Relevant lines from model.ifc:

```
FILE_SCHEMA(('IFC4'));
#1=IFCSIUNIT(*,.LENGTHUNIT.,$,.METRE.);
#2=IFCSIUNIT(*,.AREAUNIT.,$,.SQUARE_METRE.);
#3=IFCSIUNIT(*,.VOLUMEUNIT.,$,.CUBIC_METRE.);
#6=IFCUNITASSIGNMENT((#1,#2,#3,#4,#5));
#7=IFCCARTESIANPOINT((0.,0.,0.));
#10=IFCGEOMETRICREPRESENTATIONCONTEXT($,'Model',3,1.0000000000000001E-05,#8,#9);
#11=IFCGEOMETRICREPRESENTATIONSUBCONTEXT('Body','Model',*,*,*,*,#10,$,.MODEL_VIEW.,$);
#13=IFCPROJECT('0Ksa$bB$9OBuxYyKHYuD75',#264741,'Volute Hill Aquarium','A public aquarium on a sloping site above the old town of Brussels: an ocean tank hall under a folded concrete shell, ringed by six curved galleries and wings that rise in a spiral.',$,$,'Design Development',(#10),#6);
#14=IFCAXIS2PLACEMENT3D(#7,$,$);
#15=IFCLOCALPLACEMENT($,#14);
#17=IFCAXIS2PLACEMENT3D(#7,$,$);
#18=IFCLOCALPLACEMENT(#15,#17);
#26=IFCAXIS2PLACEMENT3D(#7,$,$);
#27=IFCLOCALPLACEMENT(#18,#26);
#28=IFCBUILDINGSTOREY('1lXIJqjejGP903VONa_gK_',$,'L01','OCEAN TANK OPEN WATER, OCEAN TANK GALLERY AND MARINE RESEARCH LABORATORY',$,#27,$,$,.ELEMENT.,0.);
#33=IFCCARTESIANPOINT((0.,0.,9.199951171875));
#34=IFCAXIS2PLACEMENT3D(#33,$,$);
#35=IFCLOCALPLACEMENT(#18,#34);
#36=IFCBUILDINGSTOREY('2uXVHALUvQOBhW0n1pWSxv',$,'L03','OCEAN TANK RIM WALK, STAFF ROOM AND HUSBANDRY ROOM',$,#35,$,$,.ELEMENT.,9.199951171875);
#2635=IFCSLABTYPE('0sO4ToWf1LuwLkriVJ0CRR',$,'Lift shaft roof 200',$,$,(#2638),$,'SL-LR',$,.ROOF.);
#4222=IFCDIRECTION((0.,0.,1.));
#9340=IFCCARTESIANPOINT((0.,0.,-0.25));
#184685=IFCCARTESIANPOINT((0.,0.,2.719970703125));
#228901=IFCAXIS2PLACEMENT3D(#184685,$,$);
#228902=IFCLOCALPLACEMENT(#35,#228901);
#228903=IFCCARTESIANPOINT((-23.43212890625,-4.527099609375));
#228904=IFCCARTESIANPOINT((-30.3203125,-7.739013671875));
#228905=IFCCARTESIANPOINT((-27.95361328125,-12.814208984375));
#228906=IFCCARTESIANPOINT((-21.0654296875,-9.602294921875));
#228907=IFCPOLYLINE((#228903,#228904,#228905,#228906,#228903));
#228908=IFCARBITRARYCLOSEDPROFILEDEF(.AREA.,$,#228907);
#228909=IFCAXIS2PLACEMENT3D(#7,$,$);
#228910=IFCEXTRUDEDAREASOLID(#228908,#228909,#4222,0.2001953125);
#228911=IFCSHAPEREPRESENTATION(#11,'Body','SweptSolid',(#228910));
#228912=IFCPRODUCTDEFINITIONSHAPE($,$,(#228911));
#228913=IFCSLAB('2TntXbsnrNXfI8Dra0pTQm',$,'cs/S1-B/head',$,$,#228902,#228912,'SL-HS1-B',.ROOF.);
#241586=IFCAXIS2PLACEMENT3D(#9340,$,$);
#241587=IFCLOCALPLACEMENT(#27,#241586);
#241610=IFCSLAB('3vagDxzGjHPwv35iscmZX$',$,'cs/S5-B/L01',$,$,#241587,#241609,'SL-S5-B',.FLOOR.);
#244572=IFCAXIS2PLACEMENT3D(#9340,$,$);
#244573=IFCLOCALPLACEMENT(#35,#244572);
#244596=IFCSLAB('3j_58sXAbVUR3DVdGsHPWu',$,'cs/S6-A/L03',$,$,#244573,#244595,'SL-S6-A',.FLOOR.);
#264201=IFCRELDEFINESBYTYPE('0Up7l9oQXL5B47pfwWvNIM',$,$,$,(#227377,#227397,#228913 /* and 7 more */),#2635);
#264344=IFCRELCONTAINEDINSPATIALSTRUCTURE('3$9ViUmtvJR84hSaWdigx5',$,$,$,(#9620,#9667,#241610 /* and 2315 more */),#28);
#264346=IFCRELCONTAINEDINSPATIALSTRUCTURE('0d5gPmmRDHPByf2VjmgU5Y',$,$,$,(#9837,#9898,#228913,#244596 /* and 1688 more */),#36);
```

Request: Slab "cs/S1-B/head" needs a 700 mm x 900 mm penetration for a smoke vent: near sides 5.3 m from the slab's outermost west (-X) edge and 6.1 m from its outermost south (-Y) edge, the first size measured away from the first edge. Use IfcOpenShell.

```python
import numpy as np
import ifcopenshell
import ifcopenshell.api.feature
import ifcopenshell.api.geometry
import ifcopenshell.api.root
import ifcopenshell.geom
import ifcopenshell.util.placement
import ifcopenshell.util.representation
import ifcopenshell.util.shape
import ifcopenshell.util.unit

model = ifcopenshell.open("model.ifc")
unit_scale = ifcopenshell.util.unit.calculate_unit_scale(model)
settings = ifcopenshell.geom.settings()


def volume(element):
    """Net volume in cubic metres, openings subtracted."""
    shape = ifcopenshell.geom.create_shape(settings, element)
    return ifcopenshell.util.shape.get_volume(shape.geometry)


slab = model.by_id(228913)
before = volume(slab)

# Extent in the slab's own axes, in metres. The edges named are its -X and -Y sides.
slab_shape = ifcopenshell.geom.create_shape(settings, slab)
vertices = ifcopenshell.util.shape.get_vertices(slab_shape.geometry)
x_min, y_min, bottom = vertices.min(axis=0)
top = vertices[:, 2].max()

opening = ifcopenshell.api.root.create_entity(model, ifc_class="IfcOpeningElement", name="Smoke vent opening", predefined_type="OPENING")
context = ifcopenshell.util.representation.get_context(model, "Model", "Body", "MODEL_VIEW")
width, depth = 0.7, 0.9
outline = [(0.0, 0.0), (width, 0.0), (width, depth), (0.0, depth), (0.0, 0.0)]
# Overshoot both faces by 50 mm so the cut is clean.
shape = ifcopenshell.api.geometry.add_slab_representation(
    model, context=context, depth=top - bottom + 0.1, polyline=outline
)
ifcopenshell.api.geometry.assign_representation(model, product=opening, representation=shape)

matrix = ifcopenshell.util.placement.get_local_placement(slab.ObjectPlacement)
matrix[:, 3] = matrix @ np.append(np.array([x_min + 5.3, y_min + 6.1, bottom - 0.05]) / unit_scale, 1.0)
ifcopenshell.api.geometry.edit_object_placement(model, product=opening, matrix=matrix, is_si=False)
ifcopenshell.api.feature.add_feature(model, feature=opening, element=slab)

after = volume(slab)

print(f"slab volume {before:.3f} -> {after:.3f} m3")

model.write("model_updated.ifc")
```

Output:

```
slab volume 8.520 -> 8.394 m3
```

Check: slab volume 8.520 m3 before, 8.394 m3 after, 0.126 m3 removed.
